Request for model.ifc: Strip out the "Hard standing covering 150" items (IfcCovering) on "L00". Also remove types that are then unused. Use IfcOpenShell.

First a look at what the model holds.

```python
import ifcopenshell
import ifcopenshell.util.element

model = ifcopenshell.open("model.ifc")
print(model.schema)
storey = next(s for s in model.by_type("IfcBuildingStorey") if s.Name == "L00")
coverings = [e for e in ifcopenshell.util.element.get_decomposition(storey) if e.is_a("IfcCovering")]
seen = {}
for e in coverings:
    element_type = ifcopenshell.util.element.get_type(e)
    name = element_type.Name if element_type not in (None, e) else None
    seen[name] = seen.get(name, 0) + 1
for name, count in sorted(seen.items(), key=str):
    print(count, "x", name)
```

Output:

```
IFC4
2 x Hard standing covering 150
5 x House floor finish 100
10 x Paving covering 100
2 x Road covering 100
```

```python
import ifcopenshell
import ifcopenshell.api.root
import ifcopenshell.util.element

model = ifcopenshell.open("model.ifc")

storey = next(s for s in model.by_type("IfcBuildingStorey") if s.Name == "L00")
coverings = [e for e in ifcopenshell.util.element.get_decomposition(storey) if e.is_a("IfcCovering")]
targets = [e for e in coverings if (t := ifcopenshell.util.element.get_type(e)) not in (None, e) and t.Name == "Hard standing covering 150"]
types = {ifcopenshell.util.element.get_type(e) for e in targets} - {None, *targets}

for e in targets:
    ifcopenshell.api.root.remove_product(model, product=e)
print(len(targets), "removed")

unused = [t for t in types if not ifcopenshell.util.element.get_types(t)]
for t in unused:
    ifcopenshell.api.root.remove_product(model, product=t)
print(len(unused), "unused types removed")

model.write("model_rev.ifc")
```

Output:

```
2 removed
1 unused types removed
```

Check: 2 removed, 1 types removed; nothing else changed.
